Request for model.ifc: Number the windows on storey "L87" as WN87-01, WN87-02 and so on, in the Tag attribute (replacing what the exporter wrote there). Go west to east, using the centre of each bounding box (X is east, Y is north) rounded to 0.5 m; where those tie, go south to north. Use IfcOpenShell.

First a look at what the model holds.

```python
import ifcopenshell
import ifcopenshell.util.element
import ifcopenshell.util.placement

model = ifcopenshell.open("model.ifc")
print(model.schema)
storey = next(s for s in model.by_type("IfcBuildingStorey") if s.Name == "L87")
windows = [e for e in ifcopenshell.util.element.get_decomposition(storey) if e.is_a("IfcWindow")]
for e in sorted(windows, key=lambda e: e.id()):
    origin = ifcopenshell.util.placement.get_local_placement(e.ObjectPlacement)[:3, 3]
    print(e.id(), e.Tag, e.Name, origin.round(2) + 0.0, sep=" | ")
```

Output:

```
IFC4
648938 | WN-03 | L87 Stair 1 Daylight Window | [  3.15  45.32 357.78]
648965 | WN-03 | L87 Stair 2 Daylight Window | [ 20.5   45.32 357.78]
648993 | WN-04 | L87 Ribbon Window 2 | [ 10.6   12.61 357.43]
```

```python
import ifcopenshell
import ifcopenshell.geom
import ifcopenshell.util.element
import ifcopenshell.util.shape

model = ifcopenshell.open("model.ifc")
settings = ifcopenshell.geom.settings()
settings.set("use-world-coords", True)


def centre(element):
    shape = ifcopenshell.geom.create_shape(settings, element)
    return ifcopenshell.util.shape.get_bbox_centroid(shape.geometry)


storey = next(s for s in model.by_type("IfcBuildingStorey") if s.Name == "L87")
windows = [e for e in ifcopenshell.util.element.get_decomposition(storey) if e.is_a("IfcWindow")]

# Insertion points can sit at a corner or the storey origin, so sort by the geometry (in metres).
centres = {e: centre(e) for e in windows}
windows.sort(key=lambda e: (round(centres[e][0] / 0.5), centres[e][1]))

for i, e in enumerate(windows, start=1):
    number = f"WN87-{i:02d}"
    e.Tag = number
    print(e.id(), number)

model.write("model-out.ifc")
```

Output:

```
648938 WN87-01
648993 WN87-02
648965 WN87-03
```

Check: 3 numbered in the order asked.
